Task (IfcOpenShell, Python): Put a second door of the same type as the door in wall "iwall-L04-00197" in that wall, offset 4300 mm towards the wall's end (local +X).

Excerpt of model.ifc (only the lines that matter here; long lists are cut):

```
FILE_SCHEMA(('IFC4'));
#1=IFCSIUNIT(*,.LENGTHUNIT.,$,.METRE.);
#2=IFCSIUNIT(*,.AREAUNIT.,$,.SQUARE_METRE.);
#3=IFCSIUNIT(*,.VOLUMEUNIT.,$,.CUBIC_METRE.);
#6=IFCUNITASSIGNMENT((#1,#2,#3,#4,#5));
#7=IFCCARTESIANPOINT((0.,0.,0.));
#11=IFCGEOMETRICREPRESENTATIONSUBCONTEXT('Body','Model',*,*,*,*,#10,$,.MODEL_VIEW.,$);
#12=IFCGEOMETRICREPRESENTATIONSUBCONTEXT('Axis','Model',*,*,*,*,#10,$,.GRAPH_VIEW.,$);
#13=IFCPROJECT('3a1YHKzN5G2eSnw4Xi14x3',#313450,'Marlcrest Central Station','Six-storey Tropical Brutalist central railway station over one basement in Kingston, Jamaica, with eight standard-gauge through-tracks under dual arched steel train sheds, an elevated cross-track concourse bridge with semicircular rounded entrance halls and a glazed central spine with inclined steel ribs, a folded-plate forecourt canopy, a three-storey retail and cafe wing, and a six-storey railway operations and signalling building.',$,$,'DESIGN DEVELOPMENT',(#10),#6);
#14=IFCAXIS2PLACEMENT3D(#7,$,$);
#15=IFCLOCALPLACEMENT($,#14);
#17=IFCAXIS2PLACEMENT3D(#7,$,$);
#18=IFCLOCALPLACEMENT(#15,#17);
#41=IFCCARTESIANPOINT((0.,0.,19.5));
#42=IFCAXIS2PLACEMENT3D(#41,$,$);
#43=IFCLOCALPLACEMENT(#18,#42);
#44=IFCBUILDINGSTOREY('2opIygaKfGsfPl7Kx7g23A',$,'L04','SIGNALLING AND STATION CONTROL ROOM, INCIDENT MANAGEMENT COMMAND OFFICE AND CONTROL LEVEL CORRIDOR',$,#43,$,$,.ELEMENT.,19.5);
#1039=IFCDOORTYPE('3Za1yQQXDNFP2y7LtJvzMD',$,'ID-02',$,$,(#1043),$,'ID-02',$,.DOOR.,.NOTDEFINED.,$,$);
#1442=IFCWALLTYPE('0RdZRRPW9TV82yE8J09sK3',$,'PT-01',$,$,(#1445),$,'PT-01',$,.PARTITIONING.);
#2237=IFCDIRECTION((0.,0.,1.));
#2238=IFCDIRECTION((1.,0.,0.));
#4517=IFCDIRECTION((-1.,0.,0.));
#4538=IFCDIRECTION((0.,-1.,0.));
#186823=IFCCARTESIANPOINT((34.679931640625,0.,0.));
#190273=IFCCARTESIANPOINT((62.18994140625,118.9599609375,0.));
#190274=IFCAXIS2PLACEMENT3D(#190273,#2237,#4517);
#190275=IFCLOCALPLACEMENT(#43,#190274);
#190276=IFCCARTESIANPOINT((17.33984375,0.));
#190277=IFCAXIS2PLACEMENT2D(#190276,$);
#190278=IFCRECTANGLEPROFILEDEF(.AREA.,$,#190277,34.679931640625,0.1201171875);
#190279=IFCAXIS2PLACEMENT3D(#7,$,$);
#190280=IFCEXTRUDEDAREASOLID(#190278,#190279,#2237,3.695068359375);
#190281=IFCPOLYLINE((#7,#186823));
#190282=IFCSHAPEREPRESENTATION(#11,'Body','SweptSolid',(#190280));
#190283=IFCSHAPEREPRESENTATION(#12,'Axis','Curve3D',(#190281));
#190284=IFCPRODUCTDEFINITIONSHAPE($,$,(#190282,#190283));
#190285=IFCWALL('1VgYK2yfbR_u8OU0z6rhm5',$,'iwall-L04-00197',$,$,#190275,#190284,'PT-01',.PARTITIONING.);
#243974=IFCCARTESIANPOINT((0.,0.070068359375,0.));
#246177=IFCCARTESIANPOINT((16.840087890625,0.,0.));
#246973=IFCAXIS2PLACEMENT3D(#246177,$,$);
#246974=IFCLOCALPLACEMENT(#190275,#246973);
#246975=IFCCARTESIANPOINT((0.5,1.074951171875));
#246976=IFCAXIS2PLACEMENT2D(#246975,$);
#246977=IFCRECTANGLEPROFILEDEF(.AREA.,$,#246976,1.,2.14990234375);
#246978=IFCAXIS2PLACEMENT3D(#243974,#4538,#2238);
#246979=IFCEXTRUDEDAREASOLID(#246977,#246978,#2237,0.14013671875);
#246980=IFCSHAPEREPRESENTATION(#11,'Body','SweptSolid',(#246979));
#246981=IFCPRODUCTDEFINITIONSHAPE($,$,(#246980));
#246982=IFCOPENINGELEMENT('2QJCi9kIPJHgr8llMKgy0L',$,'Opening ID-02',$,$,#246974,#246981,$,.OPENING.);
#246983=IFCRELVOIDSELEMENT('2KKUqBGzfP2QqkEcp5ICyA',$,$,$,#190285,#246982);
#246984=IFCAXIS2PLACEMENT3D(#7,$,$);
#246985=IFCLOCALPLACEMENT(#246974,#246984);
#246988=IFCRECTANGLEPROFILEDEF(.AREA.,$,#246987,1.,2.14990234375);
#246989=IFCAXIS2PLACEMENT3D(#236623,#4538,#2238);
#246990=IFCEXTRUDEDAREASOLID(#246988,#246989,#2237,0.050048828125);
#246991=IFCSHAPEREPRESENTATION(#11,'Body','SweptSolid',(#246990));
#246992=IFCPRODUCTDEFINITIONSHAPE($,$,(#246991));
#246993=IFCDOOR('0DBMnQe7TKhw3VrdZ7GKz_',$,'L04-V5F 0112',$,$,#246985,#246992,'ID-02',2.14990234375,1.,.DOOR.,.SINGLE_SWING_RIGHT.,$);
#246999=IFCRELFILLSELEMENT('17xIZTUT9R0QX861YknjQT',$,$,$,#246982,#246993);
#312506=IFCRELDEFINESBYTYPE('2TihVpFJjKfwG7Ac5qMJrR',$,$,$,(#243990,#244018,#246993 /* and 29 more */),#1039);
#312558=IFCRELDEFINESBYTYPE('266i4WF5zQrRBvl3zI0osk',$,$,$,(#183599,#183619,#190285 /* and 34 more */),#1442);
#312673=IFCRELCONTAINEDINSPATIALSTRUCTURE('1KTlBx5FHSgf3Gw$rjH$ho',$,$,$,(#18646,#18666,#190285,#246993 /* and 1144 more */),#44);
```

```python
import ifcopenshell
import ifcopenshell.api.feature
import ifcopenshell.api.geometry
import ifcopenshell.api.root
import ifcopenshell.geom
import ifcopenshell.util.element
import ifcopenshell.util.placement
import ifcopenshell.util.shape

model = ifcopenshell.open("model.ifc")
settings = ifcopenshell.geom.settings()


def volume(element):
    """Net volume in cubic metres, openings subtracted."""
    shape = ifcopenshell.geom.create_shape(settings, element)
    return ifcopenshell.util.shape.get_volume(shape.geometry)


door = model.by_guid("0DBMnQe7TKhw3VrdZ7GKz_")
opening = door.FillsVoids[0].RelatingOpeningElement
wall = opening.VoidsElements[0].RelatingBuildingElement
before = volume(wall)
shift = ifcopenshell.util.placement.get_local_placement(wall.ObjectPlacement)[:3, 0] * 4.3

# copy_class copies the void relationship, type, container and properties, but no geometry.
new_opening = ifcopenshell.api.root.copy_class(model, product=opening)
new_opening.Representation = ifcopenshell.util.element.copy_deep(
    model, opening.Representation, exclude=["IfcGeometricRepresentationContext", "IfcRepresentationMap"]
)
new_door = ifcopenshell.api.root.copy_class(model, product=door)
new_door.Representation = ifcopenshell.util.element.copy_deep(
    model, door.Representation, exclude=["IfcGeometricRepresentationContext", "IfcRepresentationMap"]
)
new_door.Tag = None
ifcopenshell.api.feature.add_filling(model, opening=new_opening, element=new_door)

for old, new in ((opening, new_opening), (door, new_door)):
    matrix = ifcopenshell.util.placement.get_local_placement(old.ObjectPlacement)
    matrix[:3, 3] += shift
    ifcopenshell.api.geometry.edit_object_placement(model, product=new, matrix=matrix, is_si=False)

after = volume(wall)

print(f"wall volume {before:.3f} -> {after:.3f} m3")

model.write("model_edited.ifc")
```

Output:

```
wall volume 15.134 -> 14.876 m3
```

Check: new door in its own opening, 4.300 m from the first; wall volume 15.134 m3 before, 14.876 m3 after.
